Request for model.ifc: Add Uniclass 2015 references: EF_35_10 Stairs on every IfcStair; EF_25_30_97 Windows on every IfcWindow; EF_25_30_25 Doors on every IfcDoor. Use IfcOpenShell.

First a look at what the model holds.

```python
import ifcopenshell

model = ifcopenshell.open("model.ifc")
print(model.schema)
print("classifications:", [c.Name for c in model.by_type("IfcClassification")])
for ifc_class in ("IfcDoor", "IfcRoof", "IfcStair", "IfcWall", "IfcWindow"):
    print(ifc_class, len(model.by_type(ifc_class)))
```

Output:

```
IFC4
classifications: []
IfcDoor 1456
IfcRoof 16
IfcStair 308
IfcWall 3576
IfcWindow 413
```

```python
import ifcopenshell
import ifcopenshell.api.classification

model = ifcopenshell.open("model.ifc")

system = ifcopenshell.api.classification.add_classification(model, classification="Uniclass 2015")

codes = {
    "IfcStair": ("EF_35_10", "Stairs"),
    "IfcWindow": ("EF_25_30_97", "Windows"),
    "IfcDoor": ("EF_25_30_25", "Doors"),
}
for ifc_class, (code, name) in codes.items():
    products = model.by_type(ifc_class)
    ifcopenshell.api.classification.add_reference(
        model, products=products, classification=system, identification=code, name=name
    )
    print(code, len(products))

model.write("model_updated.ifc")
```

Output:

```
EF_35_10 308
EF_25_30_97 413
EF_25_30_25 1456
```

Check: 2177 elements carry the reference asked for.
